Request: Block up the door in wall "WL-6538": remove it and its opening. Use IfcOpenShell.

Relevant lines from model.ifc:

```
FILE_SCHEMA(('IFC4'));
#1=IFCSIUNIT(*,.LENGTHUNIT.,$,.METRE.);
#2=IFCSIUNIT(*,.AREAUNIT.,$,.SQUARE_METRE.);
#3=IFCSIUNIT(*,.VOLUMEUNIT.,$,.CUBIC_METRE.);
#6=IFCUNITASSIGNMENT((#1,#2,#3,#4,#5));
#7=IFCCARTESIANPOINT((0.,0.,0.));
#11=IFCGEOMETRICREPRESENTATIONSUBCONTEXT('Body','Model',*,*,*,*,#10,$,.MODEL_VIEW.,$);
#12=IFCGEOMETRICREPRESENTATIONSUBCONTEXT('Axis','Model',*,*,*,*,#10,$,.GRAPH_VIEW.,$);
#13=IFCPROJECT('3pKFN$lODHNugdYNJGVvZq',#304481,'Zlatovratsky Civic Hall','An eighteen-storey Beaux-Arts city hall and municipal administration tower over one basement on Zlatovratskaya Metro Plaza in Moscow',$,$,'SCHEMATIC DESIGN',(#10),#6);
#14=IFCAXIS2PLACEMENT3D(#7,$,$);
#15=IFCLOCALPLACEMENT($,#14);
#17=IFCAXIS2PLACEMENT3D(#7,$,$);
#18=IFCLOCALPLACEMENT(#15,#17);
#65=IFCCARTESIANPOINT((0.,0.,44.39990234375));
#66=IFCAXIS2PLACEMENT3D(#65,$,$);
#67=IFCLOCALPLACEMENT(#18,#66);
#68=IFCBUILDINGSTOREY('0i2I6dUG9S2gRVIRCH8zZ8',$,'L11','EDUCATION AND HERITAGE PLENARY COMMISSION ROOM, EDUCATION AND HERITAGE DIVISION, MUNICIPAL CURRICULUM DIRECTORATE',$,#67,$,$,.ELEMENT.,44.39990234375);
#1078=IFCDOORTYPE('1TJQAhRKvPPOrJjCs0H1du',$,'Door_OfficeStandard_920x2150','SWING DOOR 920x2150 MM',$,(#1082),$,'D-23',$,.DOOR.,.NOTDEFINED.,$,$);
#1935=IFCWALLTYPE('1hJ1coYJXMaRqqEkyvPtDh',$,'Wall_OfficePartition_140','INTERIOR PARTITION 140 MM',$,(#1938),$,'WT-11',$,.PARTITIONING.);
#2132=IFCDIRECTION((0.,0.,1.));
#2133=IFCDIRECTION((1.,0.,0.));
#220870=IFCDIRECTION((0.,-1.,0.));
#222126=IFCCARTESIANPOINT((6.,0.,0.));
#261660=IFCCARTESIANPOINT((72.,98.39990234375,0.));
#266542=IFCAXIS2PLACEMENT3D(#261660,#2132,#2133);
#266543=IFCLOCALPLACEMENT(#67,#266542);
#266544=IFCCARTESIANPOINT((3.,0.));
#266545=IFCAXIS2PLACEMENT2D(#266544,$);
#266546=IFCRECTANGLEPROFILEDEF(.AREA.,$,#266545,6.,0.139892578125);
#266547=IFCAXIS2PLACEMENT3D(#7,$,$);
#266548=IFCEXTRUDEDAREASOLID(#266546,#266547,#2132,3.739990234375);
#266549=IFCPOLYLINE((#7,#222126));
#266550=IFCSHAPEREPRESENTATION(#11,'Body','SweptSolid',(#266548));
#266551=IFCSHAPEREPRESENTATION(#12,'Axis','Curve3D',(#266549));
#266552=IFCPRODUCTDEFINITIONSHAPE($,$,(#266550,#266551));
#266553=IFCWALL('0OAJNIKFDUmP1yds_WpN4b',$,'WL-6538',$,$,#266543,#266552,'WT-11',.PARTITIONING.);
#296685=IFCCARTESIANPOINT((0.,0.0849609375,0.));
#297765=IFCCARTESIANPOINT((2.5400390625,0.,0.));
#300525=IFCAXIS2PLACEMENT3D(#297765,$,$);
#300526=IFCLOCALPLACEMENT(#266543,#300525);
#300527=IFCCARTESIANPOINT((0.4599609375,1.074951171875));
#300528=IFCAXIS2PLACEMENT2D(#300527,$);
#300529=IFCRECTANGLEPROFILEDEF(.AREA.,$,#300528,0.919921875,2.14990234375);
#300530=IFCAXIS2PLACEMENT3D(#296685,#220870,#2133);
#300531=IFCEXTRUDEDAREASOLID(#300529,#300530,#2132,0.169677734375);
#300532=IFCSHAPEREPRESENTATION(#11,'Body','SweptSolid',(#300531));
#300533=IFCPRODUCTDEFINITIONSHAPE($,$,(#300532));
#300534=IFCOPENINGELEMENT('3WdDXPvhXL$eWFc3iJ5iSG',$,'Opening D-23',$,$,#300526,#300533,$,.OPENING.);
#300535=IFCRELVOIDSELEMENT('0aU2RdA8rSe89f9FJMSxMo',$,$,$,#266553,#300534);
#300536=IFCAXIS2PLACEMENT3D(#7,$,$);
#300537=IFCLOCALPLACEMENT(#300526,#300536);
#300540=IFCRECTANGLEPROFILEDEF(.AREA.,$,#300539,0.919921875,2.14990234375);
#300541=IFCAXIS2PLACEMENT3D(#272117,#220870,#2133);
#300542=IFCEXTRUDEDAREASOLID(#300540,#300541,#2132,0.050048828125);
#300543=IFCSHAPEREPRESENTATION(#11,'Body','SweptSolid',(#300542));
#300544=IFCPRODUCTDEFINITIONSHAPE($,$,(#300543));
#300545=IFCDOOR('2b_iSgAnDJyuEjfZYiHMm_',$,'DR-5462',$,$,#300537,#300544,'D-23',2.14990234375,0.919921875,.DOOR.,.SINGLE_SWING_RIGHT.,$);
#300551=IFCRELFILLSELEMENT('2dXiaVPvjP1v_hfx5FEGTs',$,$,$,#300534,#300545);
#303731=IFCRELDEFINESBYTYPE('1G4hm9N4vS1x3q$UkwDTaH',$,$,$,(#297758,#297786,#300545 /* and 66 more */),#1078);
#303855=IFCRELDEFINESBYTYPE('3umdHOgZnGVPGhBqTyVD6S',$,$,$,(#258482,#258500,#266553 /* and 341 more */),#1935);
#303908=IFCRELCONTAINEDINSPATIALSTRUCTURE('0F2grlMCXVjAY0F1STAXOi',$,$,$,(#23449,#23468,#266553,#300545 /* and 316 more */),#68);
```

```python
import ifcopenshell
import ifcopenshell.api.feature
import ifcopenshell.api.root
import ifcopenshell.geom
import ifcopenshell.util.shape

model = ifcopenshell.open("model.ifc")
settings = ifcopenshell.geom.settings()


def volume(element):
    """Net volume in cubic metres, openings subtracted."""
    shape = ifcopenshell.geom.create_shape(settings, element)
    return ifcopenshell.util.shape.get_volume(shape.geometry)


door = model.by_guid("2b_iSgAnDJyuEjfZYiHMm_")
opening = door.FillsVoids[0].RelatingOpeningElement
wall = opening.VoidsElements[0].RelatingBuildingElement
before = volume(wall)

ifcopenshell.api.root.remove_product(model, product=door)
ifcopenshell.api.feature.remove_feature(model, feature=opening)

after = volume(wall)

print(f"wall volume {before:.3f} -> {after:.3f} m3")

model.write("model_rev.ifc")
```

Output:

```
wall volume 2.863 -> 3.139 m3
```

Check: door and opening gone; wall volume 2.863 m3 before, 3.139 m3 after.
